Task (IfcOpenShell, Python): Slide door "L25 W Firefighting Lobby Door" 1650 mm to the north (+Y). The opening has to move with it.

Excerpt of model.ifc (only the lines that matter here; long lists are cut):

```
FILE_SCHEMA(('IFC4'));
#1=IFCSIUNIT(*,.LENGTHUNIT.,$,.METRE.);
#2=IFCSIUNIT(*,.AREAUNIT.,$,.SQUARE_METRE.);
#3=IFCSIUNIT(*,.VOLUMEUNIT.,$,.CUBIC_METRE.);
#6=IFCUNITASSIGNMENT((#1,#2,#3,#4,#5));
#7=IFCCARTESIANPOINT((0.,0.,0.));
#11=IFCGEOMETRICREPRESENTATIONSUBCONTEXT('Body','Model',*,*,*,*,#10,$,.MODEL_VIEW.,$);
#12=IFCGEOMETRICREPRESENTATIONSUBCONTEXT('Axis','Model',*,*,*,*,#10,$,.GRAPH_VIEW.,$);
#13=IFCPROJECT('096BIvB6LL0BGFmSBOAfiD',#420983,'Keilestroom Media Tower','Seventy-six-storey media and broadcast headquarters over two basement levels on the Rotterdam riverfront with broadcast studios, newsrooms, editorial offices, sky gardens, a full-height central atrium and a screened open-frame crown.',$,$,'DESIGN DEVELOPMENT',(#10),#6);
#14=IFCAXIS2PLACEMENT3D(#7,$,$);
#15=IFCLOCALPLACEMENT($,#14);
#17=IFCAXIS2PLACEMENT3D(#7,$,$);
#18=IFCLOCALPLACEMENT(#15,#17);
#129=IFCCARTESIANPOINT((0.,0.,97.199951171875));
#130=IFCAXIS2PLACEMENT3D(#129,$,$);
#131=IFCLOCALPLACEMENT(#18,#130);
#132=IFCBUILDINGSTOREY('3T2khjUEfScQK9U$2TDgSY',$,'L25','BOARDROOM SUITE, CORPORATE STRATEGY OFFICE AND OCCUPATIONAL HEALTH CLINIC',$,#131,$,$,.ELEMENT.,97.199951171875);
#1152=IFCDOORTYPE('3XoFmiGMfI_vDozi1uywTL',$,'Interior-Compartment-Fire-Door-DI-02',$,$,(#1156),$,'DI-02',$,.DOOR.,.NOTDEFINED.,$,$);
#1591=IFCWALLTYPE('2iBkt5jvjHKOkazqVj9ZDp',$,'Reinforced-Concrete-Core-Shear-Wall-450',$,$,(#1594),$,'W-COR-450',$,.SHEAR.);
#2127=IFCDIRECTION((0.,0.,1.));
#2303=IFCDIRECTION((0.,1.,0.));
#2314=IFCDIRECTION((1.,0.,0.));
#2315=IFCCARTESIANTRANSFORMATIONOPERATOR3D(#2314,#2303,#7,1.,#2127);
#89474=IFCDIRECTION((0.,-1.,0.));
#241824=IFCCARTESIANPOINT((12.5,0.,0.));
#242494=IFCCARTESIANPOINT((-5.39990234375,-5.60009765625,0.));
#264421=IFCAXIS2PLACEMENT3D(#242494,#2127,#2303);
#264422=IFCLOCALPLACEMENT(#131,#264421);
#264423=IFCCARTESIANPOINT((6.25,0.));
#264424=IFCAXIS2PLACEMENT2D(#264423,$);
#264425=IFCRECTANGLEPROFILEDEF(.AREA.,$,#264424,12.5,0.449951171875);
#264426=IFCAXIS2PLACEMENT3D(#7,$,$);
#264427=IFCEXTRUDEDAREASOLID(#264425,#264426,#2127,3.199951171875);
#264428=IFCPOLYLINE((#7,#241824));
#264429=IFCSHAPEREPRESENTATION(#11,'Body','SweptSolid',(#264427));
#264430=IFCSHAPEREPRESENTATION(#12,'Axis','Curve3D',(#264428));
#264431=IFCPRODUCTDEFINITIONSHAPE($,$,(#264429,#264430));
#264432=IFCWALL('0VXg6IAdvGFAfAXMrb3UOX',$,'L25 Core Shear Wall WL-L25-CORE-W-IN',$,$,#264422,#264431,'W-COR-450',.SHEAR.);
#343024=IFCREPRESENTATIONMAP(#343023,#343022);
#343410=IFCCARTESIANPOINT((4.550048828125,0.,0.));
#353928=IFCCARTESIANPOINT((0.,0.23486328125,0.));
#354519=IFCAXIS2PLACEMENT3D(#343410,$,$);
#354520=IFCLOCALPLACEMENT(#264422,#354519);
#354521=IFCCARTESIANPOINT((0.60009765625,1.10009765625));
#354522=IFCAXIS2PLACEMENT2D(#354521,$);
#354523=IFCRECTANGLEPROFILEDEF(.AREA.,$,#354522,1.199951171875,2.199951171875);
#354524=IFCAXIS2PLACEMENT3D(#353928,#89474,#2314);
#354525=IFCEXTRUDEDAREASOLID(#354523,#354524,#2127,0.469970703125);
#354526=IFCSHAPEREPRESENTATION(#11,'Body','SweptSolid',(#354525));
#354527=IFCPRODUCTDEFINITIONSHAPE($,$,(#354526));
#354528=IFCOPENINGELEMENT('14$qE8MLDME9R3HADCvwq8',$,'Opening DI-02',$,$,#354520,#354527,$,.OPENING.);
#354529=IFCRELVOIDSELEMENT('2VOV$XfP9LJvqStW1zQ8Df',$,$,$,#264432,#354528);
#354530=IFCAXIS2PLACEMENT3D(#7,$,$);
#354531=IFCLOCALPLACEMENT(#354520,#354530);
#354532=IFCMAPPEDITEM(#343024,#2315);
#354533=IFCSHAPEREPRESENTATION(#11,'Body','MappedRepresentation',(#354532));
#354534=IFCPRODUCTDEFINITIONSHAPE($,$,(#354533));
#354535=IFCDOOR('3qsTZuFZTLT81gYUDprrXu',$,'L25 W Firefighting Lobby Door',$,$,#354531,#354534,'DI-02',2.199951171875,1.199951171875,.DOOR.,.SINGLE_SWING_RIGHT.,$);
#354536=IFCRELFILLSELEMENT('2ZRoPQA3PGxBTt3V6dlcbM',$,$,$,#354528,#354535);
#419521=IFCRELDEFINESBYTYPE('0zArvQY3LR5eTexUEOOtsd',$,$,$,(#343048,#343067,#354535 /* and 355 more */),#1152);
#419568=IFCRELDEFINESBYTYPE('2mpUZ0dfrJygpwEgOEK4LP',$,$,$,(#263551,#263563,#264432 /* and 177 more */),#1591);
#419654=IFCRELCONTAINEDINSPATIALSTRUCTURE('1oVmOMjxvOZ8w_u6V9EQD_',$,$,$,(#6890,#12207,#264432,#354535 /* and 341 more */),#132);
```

```python
import ifcopenshell
import ifcopenshell.api.geometry
import ifcopenshell.util.placement
import ifcopenshell.util.unit

model = ifcopenshell.open("model.ifc")
unit_scale = ifcopenshell.util.unit.calculate_unit_scale(model)

door = model.by_guid("3qsTZuFZTLT81gYUDprrXu")
opening = door.FillsVoids[0].RelatingOpeningElement
wall = opening.VoidsElements[0].RelatingBuildingElement

wall_matrix = ifcopenshell.util.placement.get_local_placement(wall.ObjectPlacement)
shift = wall_matrix[:3, 0] * 1.65 / unit_scale
before = ifcopenshell.util.placement.get_local_placement(door.ObjectPlacement)[:3, 3].copy()

# The door is placed relative to its opening, so it follows when the opening moves.
matrix = ifcopenshell.util.placement.get_local_placement(opening.ObjectPlacement)
matrix[:3, 3] += shift
ifcopenshell.api.geometry.edit_object_placement(
    model, product=opening, matrix=matrix, is_si=False, should_transform_children=True
)

after = ifcopenshell.util.placement.get_local_placement(door.ObjectPlacement)[:3, 3]
print("door moved by", (after - before).round(3) + 0.0)

model.write("model_edited.ifc")
```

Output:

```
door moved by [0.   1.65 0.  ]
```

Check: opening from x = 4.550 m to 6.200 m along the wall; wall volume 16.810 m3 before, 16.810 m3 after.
